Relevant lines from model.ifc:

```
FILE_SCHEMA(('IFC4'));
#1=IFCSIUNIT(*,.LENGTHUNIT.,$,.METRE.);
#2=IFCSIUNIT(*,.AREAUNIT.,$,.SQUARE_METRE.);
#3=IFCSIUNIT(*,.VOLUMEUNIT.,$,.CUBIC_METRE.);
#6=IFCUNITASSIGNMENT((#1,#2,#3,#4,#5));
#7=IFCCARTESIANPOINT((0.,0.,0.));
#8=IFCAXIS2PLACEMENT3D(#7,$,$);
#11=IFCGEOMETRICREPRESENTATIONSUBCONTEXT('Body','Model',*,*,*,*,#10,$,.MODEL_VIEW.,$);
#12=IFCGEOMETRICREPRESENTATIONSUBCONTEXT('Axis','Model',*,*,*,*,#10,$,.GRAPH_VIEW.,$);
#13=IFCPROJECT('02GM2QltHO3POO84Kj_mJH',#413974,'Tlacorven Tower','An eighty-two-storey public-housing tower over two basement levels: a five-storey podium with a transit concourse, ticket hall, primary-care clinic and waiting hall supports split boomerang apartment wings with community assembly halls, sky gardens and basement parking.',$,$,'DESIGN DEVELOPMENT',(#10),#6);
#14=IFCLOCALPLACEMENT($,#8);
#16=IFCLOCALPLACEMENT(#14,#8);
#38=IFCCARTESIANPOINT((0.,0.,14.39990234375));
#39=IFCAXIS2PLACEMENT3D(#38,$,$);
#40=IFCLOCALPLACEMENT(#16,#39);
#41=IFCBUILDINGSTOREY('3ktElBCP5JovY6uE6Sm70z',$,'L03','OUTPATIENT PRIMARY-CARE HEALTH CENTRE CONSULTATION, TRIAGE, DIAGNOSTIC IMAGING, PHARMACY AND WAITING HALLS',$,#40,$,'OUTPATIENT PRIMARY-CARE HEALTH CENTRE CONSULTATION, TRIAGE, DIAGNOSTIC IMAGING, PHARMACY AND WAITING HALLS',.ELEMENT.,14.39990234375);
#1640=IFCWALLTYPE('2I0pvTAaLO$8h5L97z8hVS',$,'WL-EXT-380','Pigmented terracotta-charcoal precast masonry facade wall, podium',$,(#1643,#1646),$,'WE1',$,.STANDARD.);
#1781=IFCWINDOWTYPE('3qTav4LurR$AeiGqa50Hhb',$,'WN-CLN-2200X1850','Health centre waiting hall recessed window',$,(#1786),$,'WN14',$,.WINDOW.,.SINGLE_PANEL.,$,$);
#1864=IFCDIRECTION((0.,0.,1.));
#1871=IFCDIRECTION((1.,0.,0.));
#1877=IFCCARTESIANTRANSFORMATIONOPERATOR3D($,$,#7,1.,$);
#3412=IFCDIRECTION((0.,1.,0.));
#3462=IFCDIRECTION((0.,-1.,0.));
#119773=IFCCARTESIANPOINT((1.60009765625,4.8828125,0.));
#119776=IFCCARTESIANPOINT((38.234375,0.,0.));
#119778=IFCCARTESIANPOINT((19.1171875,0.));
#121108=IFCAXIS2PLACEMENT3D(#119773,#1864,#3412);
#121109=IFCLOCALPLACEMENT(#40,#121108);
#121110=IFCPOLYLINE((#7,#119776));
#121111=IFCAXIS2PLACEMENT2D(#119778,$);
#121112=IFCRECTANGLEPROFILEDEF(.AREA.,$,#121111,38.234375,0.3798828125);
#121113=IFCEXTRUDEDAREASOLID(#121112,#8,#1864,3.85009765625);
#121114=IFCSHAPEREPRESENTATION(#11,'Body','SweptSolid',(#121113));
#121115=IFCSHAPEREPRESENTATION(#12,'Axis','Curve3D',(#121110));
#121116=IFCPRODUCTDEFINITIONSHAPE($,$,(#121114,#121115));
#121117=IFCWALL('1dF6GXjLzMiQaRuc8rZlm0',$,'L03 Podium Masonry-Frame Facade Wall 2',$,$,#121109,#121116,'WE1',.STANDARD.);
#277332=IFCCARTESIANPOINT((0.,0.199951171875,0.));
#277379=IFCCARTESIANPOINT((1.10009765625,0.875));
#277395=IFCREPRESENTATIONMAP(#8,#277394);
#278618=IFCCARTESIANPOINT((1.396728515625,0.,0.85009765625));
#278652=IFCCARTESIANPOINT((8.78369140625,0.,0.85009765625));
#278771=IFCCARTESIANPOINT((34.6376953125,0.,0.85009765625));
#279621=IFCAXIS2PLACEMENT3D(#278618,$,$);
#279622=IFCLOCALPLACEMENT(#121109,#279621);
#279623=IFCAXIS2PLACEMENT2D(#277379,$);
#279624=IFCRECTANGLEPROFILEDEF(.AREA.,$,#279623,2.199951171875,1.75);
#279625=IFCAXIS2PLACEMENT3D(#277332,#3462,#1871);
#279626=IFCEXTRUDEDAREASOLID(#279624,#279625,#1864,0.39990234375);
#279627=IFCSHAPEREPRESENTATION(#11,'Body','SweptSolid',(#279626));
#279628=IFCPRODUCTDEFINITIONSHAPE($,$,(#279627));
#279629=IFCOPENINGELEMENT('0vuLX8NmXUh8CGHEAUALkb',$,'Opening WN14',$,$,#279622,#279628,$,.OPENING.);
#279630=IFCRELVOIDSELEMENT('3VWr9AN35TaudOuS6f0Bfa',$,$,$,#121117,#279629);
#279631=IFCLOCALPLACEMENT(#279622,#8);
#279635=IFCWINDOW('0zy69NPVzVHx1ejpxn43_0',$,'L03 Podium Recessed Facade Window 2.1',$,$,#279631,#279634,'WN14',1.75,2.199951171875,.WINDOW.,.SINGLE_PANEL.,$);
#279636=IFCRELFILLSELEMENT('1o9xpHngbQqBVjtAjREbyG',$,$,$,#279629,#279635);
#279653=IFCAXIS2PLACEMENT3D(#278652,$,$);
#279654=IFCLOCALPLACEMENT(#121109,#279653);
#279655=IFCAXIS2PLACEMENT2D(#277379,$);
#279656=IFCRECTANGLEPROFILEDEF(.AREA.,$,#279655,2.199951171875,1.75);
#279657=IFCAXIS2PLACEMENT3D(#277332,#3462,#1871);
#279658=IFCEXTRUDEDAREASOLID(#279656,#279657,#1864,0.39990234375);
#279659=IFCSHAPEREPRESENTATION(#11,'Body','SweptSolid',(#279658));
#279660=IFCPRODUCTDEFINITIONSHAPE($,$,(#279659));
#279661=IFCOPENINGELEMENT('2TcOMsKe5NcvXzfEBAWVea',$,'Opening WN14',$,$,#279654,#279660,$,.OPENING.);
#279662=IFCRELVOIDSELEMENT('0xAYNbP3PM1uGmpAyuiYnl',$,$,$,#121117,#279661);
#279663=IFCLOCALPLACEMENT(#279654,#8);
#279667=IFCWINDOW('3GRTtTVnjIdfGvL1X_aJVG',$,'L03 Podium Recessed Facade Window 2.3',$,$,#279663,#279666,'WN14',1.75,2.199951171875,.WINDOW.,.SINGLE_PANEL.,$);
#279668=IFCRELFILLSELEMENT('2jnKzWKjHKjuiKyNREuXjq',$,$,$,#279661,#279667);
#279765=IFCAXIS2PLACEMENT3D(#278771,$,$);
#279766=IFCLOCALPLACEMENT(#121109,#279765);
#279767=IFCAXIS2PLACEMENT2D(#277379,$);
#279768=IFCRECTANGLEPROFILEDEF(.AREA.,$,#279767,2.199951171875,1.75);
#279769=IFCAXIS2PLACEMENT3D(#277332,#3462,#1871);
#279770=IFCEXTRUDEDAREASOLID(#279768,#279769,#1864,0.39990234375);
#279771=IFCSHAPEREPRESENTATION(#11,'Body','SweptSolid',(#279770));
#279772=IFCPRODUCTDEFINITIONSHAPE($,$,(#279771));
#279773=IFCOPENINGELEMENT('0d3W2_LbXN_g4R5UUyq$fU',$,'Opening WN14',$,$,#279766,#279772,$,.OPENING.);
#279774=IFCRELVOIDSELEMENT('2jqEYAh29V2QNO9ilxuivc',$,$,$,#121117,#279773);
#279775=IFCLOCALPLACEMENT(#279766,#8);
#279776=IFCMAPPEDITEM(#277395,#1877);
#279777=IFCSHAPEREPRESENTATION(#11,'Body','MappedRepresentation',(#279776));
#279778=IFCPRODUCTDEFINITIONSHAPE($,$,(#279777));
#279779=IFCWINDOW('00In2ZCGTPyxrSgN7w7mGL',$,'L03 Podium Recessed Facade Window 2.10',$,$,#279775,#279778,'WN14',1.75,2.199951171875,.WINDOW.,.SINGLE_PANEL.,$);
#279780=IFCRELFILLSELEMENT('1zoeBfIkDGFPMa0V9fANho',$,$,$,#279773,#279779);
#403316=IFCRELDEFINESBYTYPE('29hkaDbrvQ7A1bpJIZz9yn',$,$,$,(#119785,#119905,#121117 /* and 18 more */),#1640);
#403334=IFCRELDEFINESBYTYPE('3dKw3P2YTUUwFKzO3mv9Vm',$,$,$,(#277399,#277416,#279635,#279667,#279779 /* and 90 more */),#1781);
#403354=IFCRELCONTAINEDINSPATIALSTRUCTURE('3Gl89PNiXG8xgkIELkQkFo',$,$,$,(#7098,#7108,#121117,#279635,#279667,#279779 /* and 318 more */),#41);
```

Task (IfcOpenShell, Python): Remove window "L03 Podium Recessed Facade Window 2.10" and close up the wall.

```python
import ifcopenshell
import ifcopenshell.api.feature
import ifcopenshell.api.root
import ifcopenshell.geom
import ifcopenshell.util.shape

model = ifcopenshell.open("model.ifc")
settings = ifcopenshell.geom.settings()


def volume(element):
    """Net volume in cubic metres, openings subtracted."""
    shape = ifcopenshell.geom.create_shape(settings, element)
    return ifcopenshell.util.shape.get_volume(shape.geometry)


window = model.by_id(279779)
opening = window.FillsVoids[0].RelatingOpeningElement
wall = opening.VoidsElements[0].RelatingBuildingElement
before = volume(wall)

ifcopenshell.api.root.remove_product(model, product=window)
ifcopenshell.api.feature.remove_feature(model, feature=opening)

after = volume(wall)

print(f"wall volume {before:.3f} -> {after:.3f} m3")

model.write("model_rev.ifc")
```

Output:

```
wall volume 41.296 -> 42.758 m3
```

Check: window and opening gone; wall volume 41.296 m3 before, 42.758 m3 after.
